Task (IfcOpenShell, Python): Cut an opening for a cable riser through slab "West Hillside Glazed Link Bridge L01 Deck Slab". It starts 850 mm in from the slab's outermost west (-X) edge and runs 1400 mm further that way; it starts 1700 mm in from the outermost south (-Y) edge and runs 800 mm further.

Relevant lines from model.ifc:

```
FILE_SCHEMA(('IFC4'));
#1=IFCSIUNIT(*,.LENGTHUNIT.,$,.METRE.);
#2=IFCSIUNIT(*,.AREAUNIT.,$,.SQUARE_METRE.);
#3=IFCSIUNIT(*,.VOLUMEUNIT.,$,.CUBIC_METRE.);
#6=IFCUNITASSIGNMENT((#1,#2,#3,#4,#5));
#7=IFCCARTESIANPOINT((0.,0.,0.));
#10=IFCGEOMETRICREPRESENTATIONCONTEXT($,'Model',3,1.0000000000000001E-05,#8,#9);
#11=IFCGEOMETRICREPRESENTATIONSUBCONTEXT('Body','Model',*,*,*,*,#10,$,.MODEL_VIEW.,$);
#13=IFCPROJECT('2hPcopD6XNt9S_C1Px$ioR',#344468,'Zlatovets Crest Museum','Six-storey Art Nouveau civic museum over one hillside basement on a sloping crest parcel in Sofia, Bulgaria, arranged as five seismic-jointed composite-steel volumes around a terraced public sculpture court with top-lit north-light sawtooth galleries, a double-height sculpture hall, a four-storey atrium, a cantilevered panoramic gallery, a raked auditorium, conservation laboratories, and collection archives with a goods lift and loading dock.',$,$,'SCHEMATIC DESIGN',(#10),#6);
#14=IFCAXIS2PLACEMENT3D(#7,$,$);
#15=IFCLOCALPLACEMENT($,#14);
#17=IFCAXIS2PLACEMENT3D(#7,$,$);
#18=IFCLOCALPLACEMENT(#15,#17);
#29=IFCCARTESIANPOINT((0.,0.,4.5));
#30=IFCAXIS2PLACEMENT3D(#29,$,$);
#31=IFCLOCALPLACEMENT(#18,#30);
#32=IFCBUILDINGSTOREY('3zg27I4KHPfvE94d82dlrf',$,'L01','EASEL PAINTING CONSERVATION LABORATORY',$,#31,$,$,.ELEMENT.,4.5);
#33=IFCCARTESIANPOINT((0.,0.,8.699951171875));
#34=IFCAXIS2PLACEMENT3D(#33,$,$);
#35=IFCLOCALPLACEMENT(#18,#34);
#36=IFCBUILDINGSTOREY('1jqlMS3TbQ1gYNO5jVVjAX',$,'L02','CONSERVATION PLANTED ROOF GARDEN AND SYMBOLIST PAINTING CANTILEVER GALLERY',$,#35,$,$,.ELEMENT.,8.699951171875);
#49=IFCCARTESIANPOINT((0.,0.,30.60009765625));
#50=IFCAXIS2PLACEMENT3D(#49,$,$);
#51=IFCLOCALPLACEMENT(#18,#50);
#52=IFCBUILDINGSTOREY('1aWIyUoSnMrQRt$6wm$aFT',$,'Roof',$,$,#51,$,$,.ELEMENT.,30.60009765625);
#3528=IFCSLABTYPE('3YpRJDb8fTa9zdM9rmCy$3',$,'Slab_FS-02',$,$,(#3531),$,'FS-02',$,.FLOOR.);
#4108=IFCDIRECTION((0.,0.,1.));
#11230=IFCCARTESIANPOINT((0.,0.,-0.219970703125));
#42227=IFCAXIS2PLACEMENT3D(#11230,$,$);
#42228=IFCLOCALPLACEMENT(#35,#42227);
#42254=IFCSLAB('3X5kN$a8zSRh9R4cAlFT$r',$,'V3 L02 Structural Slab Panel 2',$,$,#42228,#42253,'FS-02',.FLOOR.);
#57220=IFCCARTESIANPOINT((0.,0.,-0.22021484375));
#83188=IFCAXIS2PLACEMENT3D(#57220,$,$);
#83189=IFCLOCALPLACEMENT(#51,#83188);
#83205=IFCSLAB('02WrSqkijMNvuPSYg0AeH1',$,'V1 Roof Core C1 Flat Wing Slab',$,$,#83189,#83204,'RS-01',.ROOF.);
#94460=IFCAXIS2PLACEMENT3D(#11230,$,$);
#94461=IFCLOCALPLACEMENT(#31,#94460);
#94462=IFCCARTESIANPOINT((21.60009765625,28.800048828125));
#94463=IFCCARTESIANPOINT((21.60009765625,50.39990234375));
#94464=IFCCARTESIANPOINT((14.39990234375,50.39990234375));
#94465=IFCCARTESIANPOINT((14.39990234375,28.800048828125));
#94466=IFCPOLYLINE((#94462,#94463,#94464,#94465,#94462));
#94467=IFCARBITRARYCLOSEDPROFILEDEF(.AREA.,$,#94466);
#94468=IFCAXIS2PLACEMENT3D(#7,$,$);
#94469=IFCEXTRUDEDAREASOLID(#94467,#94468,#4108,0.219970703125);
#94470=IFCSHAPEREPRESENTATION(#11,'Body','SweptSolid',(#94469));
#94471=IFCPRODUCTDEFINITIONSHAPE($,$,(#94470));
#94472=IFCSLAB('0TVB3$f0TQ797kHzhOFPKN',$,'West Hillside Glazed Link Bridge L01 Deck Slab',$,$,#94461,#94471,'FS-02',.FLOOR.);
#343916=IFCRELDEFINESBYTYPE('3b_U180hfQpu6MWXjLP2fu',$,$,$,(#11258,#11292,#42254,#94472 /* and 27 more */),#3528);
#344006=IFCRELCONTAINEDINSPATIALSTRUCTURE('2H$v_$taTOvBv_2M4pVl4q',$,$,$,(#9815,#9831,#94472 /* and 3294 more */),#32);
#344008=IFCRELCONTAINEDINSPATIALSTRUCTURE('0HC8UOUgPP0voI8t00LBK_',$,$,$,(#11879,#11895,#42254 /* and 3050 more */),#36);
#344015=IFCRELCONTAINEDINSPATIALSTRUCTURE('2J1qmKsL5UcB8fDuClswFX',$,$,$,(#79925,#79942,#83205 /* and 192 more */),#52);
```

```python
import numpy as np
import ifcopenshell
import ifcopenshell.api.feature
import ifcopenshell.api.geometry
import ifcopenshell.api.root
import ifcopenshell.geom
import ifcopenshell.util.placement
import ifcopenshell.util.representation
import ifcopenshell.util.shape
import ifcopenshell.util.unit

model = ifcopenshell.open("model.ifc")
unit_scale = ifcopenshell.util.unit.calculate_unit_scale(model)
settings = ifcopenshell.geom.settings()


def volume(element):
    """Net volume in cubic metres, openings subtracted."""
    shape = ifcopenshell.geom.create_shape(settings, element)
    return ifcopenshell.util.shape.get_volume(shape.geometry)


slab = model.by_guid("0TVB3$f0TQ797kHzhOFPKN")
before = volume(slab)

# Extent in the slab's own axes, in metres. The edges named are its -X and -Y sides.
slab_shape = ifcopenshell.geom.create_shape(settings, slab)
vertices = ifcopenshell.util.shape.get_vertices(slab_shape.geometry)
x_min, y_min, bottom = vertices.min(axis=0)
top = vertices[:, 2].max()

opening = ifcopenshell.api.root.create_entity(model, ifc_class="IfcOpeningElement", name="Cable riser opening", predefined_type="OPENING")
context = ifcopenshell.util.representation.get_context(model, "Model", "Body", "MODEL_VIEW")
width, depth = 1.4, 0.8
outline = [(0.0, 0.0), (width, 0.0), (width, depth), (0.0, depth), (0.0, 0.0)]
# Overshoot both faces by 50 mm so the cut is clean.
shape = ifcopenshell.api.geometry.add_slab_representation(
    model, context=context, depth=top - bottom + 0.1, polyline=outline
)
ifcopenshell.api.geometry.assign_representation(model, product=opening, representation=shape)

matrix = ifcopenshell.util.placement.get_local_placement(slab.ObjectPlacement)
matrix[:, 3] = matrix @ np.append(np.array([x_min + 0.85, y_min + 1.7, bottom - 0.05]) / unit_scale, 1.0)
ifcopenshell.api.geometry.edit_object_placement(model, product=opening, matrix=matrix, is_si=False)
ifcopenshell.api.feature.add_feature(model, feature=opening, element=slab)

after = volume(slab)

print(f"slab volume {before:.3f} -> {after:.3f} m3")

model.write("model_edited.ifc")
```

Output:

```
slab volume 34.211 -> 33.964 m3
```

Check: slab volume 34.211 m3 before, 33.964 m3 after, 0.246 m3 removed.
